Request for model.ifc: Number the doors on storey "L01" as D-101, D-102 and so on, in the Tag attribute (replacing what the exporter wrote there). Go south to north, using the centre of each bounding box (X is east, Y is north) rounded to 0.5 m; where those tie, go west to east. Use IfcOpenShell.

First a look at what the model holds.

```python
import ifcopenshell
import ifcopenshell.util.element
import ifcopenshell.util.placement

model = ifcopenshell.open("model.ifc")
print(model.schema)
storey = next(s for s in model.by_type("IfcBuildingStorey") if s.Name == "L01")
doors = [e for e in ifcopenshell.util.element.get_decomposition(storey) if e.is_a("IfcDoor")]
for e in sorted(doors, key=lambda e: e.id()):
    origin = ifcopenshell.util.placement.get_local_placement(e.ObjectPlacement)[:3, 3]
    print(e.id(), e.Tag, e.Name, origin.round(2) + 0.0, sep=" | ")
```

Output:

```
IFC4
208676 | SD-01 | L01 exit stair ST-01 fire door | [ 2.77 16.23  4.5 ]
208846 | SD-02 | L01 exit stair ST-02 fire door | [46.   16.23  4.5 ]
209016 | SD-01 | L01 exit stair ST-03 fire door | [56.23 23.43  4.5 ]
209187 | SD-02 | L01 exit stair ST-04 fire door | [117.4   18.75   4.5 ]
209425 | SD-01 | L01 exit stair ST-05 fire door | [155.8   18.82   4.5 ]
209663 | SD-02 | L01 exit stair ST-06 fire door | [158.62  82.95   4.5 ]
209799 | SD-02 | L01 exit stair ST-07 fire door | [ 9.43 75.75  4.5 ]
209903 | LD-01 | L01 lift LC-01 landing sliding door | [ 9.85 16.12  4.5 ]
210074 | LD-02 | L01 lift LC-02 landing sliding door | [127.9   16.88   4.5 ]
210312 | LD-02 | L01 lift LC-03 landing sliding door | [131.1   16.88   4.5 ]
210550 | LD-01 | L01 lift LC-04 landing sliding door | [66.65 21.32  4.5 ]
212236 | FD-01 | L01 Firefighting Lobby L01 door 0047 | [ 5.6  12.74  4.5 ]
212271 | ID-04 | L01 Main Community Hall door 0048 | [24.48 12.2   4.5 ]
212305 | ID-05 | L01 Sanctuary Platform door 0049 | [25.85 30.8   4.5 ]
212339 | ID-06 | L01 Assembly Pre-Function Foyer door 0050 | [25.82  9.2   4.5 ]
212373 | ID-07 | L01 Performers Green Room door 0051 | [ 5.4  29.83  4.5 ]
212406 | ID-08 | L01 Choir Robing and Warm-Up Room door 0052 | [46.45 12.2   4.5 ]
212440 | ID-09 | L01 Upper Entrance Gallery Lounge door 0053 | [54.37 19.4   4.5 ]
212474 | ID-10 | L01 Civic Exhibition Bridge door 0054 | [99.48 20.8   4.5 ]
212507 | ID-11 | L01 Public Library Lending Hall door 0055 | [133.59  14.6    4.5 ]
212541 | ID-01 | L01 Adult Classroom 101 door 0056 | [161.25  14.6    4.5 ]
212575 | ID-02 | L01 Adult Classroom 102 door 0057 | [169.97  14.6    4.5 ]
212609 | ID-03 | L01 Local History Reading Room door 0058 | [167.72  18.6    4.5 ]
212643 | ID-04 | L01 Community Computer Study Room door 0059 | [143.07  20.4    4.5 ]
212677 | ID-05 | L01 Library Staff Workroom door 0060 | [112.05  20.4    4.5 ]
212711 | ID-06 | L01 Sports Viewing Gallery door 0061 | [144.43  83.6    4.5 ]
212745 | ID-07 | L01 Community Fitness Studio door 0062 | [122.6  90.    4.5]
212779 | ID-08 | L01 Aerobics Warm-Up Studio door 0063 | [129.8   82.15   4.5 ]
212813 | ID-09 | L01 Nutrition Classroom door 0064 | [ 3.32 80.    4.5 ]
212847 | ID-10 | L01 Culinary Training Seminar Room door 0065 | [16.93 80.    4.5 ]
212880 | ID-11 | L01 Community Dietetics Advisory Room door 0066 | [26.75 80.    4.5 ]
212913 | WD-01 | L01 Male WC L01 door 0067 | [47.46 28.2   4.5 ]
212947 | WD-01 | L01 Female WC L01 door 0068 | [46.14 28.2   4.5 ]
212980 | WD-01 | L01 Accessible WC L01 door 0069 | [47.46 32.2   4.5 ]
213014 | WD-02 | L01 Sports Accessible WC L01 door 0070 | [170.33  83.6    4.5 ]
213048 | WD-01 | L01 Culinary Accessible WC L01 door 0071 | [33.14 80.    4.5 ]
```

```python
import ifcopenshell
import ifcopenshell.geom
import ifcopenshell.util.element
import ifcopenshell.util.shape

model = ifcopenshell.open("model.ifc")
settings = ifcopenshell.geom.settings()
settings.set("use-world-coords", True)


def centre(element):
    shape = ifcopenshell.geom.create_shape(settings, element)
    return ifcopenshell.util.shape.get_bbox_centroid(shape.geometry)


storey = next(s for s in model.by_type("IfcBuildingStorey") if s.Name == "L01")
doors = [e for e in ifcopenshell.util.element.get_decomposition(storey) if e.is_a("IfcDoor")]

# Insertion points can sit at a corner or the storey origin, so sort by the geometry (in metres).
centres = {e: centre(e) for e in doors}
doors.sort(key=lambda e: (round(centres[e][1] / 0.5), centres[e][0]))

for i, e in enumerate(doors, start=1):
    number = f"D-1{i:02d}"
    e.Tag = number
    print(e.id(), number)

model.write("model_updated.ifc")
```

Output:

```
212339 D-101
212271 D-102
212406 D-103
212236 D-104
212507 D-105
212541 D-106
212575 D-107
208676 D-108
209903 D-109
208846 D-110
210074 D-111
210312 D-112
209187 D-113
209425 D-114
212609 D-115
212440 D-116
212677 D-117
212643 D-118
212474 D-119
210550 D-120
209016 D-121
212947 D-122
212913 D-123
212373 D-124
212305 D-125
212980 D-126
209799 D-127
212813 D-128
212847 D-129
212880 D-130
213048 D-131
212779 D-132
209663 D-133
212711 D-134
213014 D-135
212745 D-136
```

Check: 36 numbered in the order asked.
